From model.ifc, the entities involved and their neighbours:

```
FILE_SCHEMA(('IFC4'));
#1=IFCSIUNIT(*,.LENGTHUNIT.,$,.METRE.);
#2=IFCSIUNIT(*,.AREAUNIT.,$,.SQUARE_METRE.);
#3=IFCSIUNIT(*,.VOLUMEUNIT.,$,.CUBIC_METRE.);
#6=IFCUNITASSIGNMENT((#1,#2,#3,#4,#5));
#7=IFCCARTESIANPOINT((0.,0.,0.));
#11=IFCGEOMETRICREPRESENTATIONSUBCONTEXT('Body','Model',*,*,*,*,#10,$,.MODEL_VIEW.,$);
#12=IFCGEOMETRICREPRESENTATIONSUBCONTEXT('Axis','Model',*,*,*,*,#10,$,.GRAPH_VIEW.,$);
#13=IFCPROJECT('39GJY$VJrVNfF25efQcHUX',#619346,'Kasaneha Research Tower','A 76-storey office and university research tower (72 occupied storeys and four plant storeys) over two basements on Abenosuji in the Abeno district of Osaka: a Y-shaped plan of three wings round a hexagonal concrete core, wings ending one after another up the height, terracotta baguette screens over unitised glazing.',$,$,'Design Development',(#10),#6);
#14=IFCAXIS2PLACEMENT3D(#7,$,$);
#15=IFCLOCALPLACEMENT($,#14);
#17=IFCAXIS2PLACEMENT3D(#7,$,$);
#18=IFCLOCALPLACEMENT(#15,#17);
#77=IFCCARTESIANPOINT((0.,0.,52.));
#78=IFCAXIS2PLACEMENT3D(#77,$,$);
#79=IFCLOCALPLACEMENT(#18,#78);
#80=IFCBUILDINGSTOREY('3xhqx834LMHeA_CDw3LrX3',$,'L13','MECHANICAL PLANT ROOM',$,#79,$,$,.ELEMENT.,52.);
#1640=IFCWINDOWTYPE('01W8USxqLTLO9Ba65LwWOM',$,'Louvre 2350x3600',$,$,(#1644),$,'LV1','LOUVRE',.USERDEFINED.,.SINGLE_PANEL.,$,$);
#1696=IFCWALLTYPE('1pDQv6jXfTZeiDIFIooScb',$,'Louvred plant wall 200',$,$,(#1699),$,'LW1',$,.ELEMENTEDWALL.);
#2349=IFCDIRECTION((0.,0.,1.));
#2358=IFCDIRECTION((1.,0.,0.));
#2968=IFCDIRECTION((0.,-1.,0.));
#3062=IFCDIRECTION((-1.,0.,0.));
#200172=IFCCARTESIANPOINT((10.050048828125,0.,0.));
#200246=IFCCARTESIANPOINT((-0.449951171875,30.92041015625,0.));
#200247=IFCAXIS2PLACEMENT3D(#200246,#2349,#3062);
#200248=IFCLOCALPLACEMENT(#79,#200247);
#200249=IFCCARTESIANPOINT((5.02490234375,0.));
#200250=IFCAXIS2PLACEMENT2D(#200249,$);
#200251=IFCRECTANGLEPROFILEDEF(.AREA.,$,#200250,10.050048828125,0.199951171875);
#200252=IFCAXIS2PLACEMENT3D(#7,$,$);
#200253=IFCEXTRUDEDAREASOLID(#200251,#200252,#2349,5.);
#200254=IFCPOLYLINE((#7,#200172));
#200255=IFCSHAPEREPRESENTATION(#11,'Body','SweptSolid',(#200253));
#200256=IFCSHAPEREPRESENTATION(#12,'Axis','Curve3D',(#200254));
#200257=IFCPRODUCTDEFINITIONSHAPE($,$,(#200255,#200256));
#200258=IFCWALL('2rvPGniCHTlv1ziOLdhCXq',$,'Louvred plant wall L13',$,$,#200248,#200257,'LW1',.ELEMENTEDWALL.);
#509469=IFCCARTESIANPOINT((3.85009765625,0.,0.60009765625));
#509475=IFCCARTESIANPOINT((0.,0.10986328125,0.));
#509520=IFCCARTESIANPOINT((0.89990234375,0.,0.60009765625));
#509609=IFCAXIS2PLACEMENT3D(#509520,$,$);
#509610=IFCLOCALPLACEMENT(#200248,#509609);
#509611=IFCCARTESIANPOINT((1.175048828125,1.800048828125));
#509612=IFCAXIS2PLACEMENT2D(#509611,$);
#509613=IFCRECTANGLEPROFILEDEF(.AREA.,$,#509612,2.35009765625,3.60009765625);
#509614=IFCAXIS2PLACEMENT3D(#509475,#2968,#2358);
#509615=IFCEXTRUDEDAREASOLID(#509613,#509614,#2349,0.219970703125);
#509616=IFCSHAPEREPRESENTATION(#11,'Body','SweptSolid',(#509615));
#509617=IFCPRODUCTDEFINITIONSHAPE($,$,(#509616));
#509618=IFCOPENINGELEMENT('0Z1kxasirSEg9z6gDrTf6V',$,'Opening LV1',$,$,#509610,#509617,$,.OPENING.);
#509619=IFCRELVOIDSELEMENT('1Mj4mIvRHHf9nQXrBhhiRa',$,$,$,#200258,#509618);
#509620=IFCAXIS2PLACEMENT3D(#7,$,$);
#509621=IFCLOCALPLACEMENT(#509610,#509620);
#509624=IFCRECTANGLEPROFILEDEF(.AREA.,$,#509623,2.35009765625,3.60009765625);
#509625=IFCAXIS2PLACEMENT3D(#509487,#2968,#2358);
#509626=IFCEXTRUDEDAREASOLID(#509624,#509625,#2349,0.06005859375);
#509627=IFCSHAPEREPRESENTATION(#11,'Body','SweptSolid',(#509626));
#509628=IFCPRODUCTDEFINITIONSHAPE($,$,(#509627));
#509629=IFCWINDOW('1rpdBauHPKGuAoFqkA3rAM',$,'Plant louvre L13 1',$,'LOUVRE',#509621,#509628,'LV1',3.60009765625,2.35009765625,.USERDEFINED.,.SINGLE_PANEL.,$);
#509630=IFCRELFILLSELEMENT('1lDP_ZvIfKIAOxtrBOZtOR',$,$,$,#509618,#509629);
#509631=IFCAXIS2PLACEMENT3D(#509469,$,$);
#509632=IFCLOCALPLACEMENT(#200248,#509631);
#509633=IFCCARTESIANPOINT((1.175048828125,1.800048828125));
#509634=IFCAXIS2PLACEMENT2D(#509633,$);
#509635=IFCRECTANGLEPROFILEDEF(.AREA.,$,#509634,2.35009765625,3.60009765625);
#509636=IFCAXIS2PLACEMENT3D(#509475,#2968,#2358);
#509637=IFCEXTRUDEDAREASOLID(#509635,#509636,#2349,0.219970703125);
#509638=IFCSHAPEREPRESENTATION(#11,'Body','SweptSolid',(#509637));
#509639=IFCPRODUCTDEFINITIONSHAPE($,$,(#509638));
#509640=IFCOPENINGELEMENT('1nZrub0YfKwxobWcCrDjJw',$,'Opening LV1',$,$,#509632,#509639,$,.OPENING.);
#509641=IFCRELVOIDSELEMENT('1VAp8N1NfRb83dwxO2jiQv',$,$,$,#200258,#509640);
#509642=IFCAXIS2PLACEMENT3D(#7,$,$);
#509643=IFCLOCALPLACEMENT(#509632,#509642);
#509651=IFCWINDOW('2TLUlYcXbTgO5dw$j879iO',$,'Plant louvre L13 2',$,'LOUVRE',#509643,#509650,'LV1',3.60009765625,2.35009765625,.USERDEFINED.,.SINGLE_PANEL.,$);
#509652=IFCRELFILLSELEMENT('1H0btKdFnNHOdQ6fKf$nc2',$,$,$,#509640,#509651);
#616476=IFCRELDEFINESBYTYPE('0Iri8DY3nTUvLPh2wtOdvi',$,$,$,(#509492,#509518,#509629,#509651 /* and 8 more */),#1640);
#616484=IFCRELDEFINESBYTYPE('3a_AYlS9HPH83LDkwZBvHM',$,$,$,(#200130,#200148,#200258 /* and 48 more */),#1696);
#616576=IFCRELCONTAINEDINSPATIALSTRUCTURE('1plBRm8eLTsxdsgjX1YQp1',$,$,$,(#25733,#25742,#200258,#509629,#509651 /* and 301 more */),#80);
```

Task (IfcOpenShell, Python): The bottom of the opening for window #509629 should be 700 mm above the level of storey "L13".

```python
import numpy as np
import ifcopenshell
import ifcopenshell.api.geometry
import ifcopenshell.geom
import ifcopenshell.util.element
import ifcopenshell.util.placement
import ifcopenshell.util.shape
import ifcopenshell.util.unit

model = ifcopenshell.open("model.ifc")
unit_scale = ifcopenshell.util.unit.calculate_unit_scale(model)

window = model.by_guid("1rpdBauHPKGuAoFqkA3rAM")
opening = window.FillsVoids[0].RelatingOpeningElement
storey = ifcopenshell.util.element.get_container(window, ifc_class="IfcBuildingStorey")
level = ifcopenshell.util.placement.get_local_placement(storey.ObjectPlacement)[2, 3]

# The opening's origin need not be at the sill, so measure its lowest point.
shape = ifcopenshell.geom.create_shape(ifcopenshell.geom.settings(), opening)
bottom = ifcopenshell.util.shape.get_shape_bottom_elevation(shape, shape.geometry) / unit_scale
dz = level + 0.7 / unit_scale - bottom

shift = np.array([0.0, 0.0, dz])
# The window is placed relative to its opening, so it follows when the opening moves.
matrix = ifcopenshell.util.placement.get_local_placement(opening.ObjectPlacement)
matrix[:3, 3] += shift
ifcopenshell.api.geometry.edit_object_placement(
    model, product=opening, matrix=matrix, is_si=False, should_transform_children=True
)

print(f"moved by {dz * unit_scale:+.3f} m")

model.write("model_v2.ifc")
```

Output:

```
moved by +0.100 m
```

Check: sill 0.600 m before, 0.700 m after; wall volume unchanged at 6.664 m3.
